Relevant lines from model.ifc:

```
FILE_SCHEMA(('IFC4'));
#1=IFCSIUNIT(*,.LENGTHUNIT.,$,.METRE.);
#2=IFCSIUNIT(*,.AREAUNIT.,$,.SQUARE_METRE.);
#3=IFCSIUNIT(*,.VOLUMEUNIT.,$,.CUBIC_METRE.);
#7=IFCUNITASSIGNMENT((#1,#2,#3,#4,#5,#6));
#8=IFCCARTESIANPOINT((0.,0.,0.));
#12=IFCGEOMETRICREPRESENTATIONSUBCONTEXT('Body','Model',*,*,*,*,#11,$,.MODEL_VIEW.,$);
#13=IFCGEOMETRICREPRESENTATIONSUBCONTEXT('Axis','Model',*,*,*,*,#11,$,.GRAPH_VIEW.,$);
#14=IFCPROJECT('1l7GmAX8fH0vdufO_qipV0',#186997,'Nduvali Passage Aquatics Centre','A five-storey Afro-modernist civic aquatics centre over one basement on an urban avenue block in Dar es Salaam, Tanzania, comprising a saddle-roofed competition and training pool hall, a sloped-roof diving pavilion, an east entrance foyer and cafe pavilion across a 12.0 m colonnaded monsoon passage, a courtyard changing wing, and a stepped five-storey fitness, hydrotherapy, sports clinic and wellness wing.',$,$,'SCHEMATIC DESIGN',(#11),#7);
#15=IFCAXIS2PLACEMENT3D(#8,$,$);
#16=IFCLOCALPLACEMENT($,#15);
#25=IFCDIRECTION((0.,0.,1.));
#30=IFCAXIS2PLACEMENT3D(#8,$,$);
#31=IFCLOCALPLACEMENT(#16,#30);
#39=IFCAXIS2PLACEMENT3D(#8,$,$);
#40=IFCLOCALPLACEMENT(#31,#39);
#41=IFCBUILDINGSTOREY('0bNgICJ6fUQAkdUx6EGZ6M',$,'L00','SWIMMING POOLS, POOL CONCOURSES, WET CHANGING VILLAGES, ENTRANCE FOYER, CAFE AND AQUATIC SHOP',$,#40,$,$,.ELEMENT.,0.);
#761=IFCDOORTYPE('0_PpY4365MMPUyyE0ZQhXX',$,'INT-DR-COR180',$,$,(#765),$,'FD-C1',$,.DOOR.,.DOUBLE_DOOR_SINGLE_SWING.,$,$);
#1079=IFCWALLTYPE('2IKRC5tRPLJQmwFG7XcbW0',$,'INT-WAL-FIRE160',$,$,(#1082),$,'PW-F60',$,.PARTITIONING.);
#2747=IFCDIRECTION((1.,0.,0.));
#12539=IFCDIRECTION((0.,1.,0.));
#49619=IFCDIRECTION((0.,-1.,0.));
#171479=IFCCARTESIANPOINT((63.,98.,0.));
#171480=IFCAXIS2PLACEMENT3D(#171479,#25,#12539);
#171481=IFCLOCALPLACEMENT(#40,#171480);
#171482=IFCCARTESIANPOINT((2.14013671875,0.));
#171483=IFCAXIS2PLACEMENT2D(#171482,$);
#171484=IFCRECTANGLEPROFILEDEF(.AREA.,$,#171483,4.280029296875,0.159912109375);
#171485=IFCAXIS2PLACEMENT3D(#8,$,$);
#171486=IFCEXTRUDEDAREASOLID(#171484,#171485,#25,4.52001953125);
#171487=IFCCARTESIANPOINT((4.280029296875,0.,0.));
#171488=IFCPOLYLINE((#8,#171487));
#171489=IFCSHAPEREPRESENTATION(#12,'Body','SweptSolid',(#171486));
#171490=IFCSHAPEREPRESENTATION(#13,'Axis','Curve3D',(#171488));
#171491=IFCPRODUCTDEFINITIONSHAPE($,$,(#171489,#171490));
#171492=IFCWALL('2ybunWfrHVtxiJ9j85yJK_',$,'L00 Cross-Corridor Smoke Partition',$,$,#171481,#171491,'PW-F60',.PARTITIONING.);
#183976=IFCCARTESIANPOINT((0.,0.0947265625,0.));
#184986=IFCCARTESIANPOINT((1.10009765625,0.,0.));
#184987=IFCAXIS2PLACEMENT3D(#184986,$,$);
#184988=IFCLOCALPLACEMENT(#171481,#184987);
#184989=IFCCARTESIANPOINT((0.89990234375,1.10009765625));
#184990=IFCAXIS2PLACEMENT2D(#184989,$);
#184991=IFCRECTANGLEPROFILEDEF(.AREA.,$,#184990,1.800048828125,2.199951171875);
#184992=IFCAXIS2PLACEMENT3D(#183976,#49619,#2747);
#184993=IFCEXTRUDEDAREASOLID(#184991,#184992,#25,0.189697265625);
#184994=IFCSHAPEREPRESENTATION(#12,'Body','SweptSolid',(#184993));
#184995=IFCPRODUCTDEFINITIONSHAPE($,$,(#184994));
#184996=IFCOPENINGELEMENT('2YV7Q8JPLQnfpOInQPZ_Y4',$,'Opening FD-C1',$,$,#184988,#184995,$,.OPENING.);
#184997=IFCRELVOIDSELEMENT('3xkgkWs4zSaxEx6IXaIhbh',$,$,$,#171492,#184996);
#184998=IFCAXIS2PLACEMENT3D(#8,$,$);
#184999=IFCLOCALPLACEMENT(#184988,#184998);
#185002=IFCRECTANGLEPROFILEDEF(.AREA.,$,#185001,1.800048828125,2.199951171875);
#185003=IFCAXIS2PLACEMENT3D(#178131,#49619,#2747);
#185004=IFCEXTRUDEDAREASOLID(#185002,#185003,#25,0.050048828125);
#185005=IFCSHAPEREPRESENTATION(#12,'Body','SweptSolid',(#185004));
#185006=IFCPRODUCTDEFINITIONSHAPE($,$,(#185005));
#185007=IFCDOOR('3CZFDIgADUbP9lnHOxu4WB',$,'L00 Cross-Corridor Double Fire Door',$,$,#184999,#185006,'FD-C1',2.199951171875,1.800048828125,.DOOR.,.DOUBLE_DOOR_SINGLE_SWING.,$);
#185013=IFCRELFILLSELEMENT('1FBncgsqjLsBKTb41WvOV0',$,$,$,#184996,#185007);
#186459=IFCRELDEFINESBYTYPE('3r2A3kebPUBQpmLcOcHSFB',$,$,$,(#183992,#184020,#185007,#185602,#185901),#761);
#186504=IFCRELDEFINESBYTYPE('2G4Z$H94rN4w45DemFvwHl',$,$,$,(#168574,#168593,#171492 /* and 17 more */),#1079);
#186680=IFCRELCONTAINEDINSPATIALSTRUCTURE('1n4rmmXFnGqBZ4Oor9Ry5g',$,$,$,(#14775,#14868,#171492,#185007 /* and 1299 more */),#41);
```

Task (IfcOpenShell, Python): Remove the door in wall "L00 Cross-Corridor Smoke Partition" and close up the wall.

```python
import ifcopenshell
import ifcopenshell.api.feature
import ifcopenshell.api.root
import ifcopenshell.geom
import ifcopenshell.util.shape

model = ifcopenshell.open("model.ifc")
settings = ifcopenshell.geom.settings()


def volume(element):
    """Net volume in cubic metres, openings subtracted."""
    shape = ifcopenshell.geom.create_shape(settings, element)
    return ifcopenshell.util.shape.get_volume(shape.geometry)


door = model.by_id(185007)
opening = door.FillsVoids[0].RelatingOpeningElement
wall = opening.VoidsElements[0].RelatingBuildingElement
before = volume(wall)

ifcopenshell.api.root.remove_product(model, product=door)
ifcopenshell.api.feature.remove_feature(model, feature=opening)

after = volume(wall)

print(f"wall volume {before:.3f} -> {after:.3f} m3")

model.write("model_v2.ifc")
```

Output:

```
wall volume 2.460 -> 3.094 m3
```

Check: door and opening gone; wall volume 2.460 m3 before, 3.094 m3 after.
